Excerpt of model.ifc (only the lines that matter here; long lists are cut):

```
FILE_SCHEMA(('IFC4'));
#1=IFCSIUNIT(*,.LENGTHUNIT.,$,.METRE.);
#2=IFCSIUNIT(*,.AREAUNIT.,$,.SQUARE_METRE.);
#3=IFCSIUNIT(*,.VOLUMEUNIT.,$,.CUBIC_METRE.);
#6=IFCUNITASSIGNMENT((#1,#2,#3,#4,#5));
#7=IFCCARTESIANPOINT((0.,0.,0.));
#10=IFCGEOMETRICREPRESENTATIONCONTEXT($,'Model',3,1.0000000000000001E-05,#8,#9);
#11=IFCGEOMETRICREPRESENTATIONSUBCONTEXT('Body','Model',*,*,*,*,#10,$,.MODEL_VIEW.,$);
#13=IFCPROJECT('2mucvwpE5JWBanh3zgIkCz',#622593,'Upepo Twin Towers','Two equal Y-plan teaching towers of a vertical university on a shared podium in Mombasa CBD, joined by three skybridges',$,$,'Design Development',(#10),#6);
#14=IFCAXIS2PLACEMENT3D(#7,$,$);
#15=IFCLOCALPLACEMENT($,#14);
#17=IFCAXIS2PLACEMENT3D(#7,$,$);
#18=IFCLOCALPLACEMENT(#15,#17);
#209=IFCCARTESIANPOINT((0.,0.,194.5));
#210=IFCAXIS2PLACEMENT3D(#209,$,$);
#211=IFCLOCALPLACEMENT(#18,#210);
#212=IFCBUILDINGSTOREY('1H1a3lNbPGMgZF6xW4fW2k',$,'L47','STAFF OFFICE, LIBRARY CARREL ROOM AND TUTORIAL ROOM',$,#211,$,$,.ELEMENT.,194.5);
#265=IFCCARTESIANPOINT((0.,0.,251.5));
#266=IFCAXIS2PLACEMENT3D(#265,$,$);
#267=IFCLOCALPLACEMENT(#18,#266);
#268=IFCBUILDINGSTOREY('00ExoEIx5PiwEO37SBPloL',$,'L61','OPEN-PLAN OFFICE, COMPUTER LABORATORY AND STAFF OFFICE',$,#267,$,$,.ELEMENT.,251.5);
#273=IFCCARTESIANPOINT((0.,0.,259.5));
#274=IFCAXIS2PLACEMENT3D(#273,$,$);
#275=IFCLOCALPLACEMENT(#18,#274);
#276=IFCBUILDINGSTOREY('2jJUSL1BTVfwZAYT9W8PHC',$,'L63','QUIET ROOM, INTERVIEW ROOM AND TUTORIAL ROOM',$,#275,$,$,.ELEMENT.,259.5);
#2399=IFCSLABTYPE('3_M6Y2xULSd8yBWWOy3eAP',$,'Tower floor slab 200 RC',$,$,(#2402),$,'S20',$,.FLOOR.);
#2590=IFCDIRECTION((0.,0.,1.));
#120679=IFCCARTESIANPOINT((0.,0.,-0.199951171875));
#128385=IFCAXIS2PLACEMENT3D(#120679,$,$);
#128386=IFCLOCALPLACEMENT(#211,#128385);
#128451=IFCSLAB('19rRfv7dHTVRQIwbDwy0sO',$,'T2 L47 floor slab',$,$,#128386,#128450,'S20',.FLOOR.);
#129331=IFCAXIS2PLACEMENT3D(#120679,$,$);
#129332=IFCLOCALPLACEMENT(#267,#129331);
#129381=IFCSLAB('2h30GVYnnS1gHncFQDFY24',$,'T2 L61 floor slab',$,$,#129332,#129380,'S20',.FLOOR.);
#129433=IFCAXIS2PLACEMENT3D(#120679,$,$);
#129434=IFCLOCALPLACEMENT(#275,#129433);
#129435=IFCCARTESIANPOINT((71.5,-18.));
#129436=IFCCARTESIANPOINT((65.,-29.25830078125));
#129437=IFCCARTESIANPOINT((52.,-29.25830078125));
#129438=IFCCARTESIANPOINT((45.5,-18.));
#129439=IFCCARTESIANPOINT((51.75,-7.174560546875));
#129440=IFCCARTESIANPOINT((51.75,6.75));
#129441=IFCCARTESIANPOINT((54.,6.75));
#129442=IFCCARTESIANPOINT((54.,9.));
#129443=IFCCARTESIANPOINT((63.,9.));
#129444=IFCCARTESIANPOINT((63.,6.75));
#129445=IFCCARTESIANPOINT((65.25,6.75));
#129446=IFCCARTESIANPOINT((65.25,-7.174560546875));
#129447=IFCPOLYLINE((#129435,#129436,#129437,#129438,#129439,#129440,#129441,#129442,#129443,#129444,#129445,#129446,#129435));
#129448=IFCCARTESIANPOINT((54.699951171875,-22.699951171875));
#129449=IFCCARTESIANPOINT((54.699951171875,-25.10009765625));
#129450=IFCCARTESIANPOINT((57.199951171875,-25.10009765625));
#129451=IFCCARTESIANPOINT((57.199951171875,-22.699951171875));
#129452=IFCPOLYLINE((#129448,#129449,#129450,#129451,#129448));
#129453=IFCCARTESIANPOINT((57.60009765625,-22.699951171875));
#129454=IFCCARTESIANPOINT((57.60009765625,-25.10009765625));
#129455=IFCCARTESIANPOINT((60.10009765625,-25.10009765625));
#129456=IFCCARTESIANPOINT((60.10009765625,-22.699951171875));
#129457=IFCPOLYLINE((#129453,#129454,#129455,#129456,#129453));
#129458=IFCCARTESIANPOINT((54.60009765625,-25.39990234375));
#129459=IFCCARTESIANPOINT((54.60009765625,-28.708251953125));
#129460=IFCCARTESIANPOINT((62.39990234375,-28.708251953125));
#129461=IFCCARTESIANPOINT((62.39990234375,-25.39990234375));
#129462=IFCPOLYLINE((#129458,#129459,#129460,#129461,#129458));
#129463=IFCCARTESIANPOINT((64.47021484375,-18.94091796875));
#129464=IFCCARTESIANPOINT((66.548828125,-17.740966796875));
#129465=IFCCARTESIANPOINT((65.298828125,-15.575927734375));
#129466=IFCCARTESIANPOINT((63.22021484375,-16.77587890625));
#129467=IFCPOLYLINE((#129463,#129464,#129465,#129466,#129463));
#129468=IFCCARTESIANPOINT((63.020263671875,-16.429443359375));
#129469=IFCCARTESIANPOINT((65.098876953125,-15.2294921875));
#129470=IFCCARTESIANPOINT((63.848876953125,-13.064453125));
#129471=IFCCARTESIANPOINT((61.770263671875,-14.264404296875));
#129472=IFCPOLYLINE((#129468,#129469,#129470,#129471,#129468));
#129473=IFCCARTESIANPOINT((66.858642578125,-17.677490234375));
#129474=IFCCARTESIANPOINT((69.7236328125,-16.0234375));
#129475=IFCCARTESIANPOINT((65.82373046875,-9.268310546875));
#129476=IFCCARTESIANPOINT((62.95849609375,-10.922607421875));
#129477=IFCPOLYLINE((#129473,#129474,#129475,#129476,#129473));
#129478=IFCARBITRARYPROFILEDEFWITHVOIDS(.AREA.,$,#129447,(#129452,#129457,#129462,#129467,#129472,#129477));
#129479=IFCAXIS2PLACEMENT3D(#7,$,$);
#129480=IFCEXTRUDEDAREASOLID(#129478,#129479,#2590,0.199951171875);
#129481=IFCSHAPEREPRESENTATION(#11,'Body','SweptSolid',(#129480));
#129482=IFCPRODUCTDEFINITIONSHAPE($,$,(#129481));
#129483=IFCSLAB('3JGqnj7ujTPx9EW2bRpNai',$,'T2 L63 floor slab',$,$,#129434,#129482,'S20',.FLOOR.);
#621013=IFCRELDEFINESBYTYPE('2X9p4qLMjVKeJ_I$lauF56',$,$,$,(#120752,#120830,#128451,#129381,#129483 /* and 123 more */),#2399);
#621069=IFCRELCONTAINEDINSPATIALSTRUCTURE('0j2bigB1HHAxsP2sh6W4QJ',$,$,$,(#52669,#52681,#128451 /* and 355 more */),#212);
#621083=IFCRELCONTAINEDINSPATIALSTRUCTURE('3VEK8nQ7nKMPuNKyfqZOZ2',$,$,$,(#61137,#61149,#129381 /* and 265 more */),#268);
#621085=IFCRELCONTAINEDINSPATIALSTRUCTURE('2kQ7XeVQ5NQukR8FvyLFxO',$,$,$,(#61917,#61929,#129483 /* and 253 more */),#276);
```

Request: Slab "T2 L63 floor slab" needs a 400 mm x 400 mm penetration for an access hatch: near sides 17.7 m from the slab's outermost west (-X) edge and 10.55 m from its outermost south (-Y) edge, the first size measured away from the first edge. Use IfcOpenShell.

```python
import numpy as np
import ifcopenshell
import ifcopenshell.api.feature
import ifcopenshell.api.geometry
import ifcopenshell.api.root
import ifcopenshell.geom
import ifcopenshell.util.placement
import ifcopenshell.util.representation
import ifcopenshell.util.shape
import ifcopenshell.util.unit

model = ifcopenshell.open("model.ifc")
unit_scale = ifcopenshell.util.unit.calculate_unit_scale(model)
settings = ifcopenshell.geom.settings()


def volume(element):
    """Net volume in cubic metres, openings subtracted."""
    shape = ifcopenshell.geom.create_shape(settings, element)
    return ifcopenshell.util.shape.get_volume(shape.geometry)


slab = model.by_guid("3JGqnj7ujTPx9EW2bRpNai")
before = volume(slab)

# Extent in the slab's own axes, in metres. The edges named are its -X and -Y sides.
slab_shape = ifcopenshell.geom.create_shape(settings, slab)
vertices = ifcopenshell.util.shape.get_vertices(slab_shape.geometry)
x_min, y_min, bottom = vertices.min(axis=0)
top = vertices[:, 2].max()

opening = ifcopenshell.api.root.create_entity(model, ifc_class="IfcOpeningElement", name="Access hatch opening", predefined_type="OPENING")
context = ifcopenshell.util.representation.get_context(model, "Model", "Body", "MODEL_VIEW")
width, depth = 0.4, 0.4
outline = [(0.0, 0.0), (width, 0.0), (width, depth), (0.0, depth), (0.0, 0.0)]
# Overshoot both faces by 50 mm so the cut is clean.
shape = ifcopenshell.api.geometry.add_slab_representation(
    model, context=context, depth=top - bottom + 0.1, polyline=outline
)
ifcopenshell.api.geometry.assign_representation(model, product=opening, representation=shape)

matrix = ifcopenshell.util.placement.get_local_placement(slab.ObjectPlacement)
matrix[:, 3] = matrix @ np.append(np.array([x_min + 17.7, y_min + 10.55, bottom - 0.05]) / unit_scale, 1.0)
ifcopenshell.api.geometry.edit_object_placement(model, product=opening, matrix=matrix, is_si=False)
ifcopenshell.api.feature.add_feature(model, feature=opening, element=slab)

after = volume(slab)

print(f"slab volume {before:.3f} -> {after:.3f} m3")

model.write("model_v2.ifc")
```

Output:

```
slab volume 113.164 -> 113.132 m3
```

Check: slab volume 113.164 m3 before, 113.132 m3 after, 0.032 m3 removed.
